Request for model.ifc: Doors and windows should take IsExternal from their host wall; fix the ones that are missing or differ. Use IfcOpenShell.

First a look at what the model holds.

```python
import ifcopenshell
import ifcopenshell.util.element

model = ifcopenshell.open("model.ifc")
print(model.schema)
seen = {}
for e in model.by_type("IfcDoor") + model.by_type("IfcWindow"):
    if not e.FillsVoids:
        continue
    host = e.FillsVoids[0].RelatingOpeningElement.VoidsElements[0].RelatingBuildingElement
    own = ifcopenshell.util.element.get_pset(e, f"Pset_{e.is_a()[3:].removesuffix('StandardCase')}Common", "IsExternal")
    wall = ifcopenshell.util.element.get_pset(host, "Pset_WallCommon", "IsExternal")
    seen[e.is_a(), own, wall] = seen.get((e.is_a(), own, wall), 0) + 1
for (cls, own, wall), count in sorted(seen.items(), key=str):
    print(count, cls, "IsExternal:", own, "| host wall:", wall)
```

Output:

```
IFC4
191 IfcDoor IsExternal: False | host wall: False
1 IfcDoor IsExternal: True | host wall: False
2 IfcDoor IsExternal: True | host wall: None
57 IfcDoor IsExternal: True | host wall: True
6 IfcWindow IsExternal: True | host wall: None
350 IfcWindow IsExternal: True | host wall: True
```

```python
import ifcopenshell
import ifcopenshell.api.pset
import ifcopenshell.util.element

model = ifcopenshell.open("model.ifc")

count = 0
for ifc_class, pset_name in (("IfcDoor", "Pset_DoorCommon"), ("IfcWindow", "Pset_WindowCommon")):
    for e in model.by_type(ifc_class):
        if not e.FillsVoids:
            continue
        host = e.FillsVoids[0].RelatingOpeningElement.VoidsElements[0].RelatingBuildingElement
        external = ifcopenshell.util.element.get_pset(host, "Pset_WallCommon", "IsExternal")
        if external is None or ifcopenshell.util.element.get_pset(e, pset_name, "IsExternal") == external:
            continue
        pset = ifcopenshell.api.pset.add_pset(model, product=e, name=pset_name)
        ifcopenshell.api.pset.edit_pset(model, pset=pset, properties={"IsExternal": external})
        count += 1

print(count, "updated")

model.write("model_edited.ifc")
```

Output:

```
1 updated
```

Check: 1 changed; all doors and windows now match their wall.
